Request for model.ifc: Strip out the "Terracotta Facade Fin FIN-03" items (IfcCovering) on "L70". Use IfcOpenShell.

First a look at what the model holds.

```python
import ifcopenshell
import ifcopenshell.util.element

model = ifcopenshell.open("model.ifc")
print(model.schema)
storey = next(s for s in model.by_type("IfcBuildingStorey") if s.Name == "L70")
coverings = [e for e in ifcopenshell.util.element.get_decomposition(storey) if e.is_a("IfcCovering")]
seen = {}
for e in coverings:
    element_type = ifcopenshell.util.element.get_type(e)
    name = element_type.Name if element_type not in (None, e) else None
    seen[name] = seen.get(name, 0) + 1
for name, count in sorted(seen.items(), key=str):
    print(count, "x", name)
```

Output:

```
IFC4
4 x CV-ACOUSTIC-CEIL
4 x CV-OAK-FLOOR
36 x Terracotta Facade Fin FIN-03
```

```python
import ifcopenshell
import ifcopenshell.api.root
import ifcopenshell.util.element

model = ifcopenshell.open("model.ifc")

storey = next(s for s in model.by_type("IfcBuildingStorey") if s.Name == "L70")
coverings = [e for e in ifcopenshell.util.element.get_decomposition(storey) if e.is_a("IfcCovering")]
targets = [e for e in coverings if (t := ifcopenshell.util.element.get_type(e)) not in (None, e) and t.Name == "Terracotta Facade Fin FIN-03"]

for e in targets:
    ifcopenshell.api.root.remove_product(model, product=e)
print(len(targets), "removed")

model.write("model_updated.ifc")
```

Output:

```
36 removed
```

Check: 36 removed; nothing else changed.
